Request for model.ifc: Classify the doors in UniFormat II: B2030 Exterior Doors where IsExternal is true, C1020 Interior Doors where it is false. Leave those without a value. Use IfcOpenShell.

First a look at what the model holds.

```python
import ifcopenshell
import ifcopenshell.util.element

model = ifcopenshell.open("model.ifc")
print(model.schema)
print("classifications:", [c.Name for c in model.by_type("IfcClassification")])
values = [ifcopenshell.util.element.get_pset(e, "Pset_DoorCommon", "IsExternal") for e in model.by_type("IfcDoor")]
for value in (True, False, None):
    print("IsExternal", value, values.count(value))
```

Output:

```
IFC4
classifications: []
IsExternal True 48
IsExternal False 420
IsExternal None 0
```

```python
import ifcopenshell
import ifcopenshell.api.classification
import ifcopenshell.util.element

model = ifcopenshell.open("model.ifc")

system = ifcopenshell.api.classification.add_classification(model, classification="UniFormat II")

doors = model.by_type("IfcDoor")
external = {e: ifcopenshell.util.element.get_pset(e, "Pset_DoorCommon", "IsExternal") for e in doors}
for flag, code, name in ((True, "B2030", "Exterior Doors"), (False, "C1020", "Interior Doors")):
    products = [e for e in doors if external[e] is flag]
    ifcopenshell.api.classification.add_reference(
        model, products=products, classification=system, identification=code, name=name
    )
    print(code, len(products))

model.write("model_edited.ifc")
```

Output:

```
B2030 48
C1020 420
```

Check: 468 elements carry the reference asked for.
